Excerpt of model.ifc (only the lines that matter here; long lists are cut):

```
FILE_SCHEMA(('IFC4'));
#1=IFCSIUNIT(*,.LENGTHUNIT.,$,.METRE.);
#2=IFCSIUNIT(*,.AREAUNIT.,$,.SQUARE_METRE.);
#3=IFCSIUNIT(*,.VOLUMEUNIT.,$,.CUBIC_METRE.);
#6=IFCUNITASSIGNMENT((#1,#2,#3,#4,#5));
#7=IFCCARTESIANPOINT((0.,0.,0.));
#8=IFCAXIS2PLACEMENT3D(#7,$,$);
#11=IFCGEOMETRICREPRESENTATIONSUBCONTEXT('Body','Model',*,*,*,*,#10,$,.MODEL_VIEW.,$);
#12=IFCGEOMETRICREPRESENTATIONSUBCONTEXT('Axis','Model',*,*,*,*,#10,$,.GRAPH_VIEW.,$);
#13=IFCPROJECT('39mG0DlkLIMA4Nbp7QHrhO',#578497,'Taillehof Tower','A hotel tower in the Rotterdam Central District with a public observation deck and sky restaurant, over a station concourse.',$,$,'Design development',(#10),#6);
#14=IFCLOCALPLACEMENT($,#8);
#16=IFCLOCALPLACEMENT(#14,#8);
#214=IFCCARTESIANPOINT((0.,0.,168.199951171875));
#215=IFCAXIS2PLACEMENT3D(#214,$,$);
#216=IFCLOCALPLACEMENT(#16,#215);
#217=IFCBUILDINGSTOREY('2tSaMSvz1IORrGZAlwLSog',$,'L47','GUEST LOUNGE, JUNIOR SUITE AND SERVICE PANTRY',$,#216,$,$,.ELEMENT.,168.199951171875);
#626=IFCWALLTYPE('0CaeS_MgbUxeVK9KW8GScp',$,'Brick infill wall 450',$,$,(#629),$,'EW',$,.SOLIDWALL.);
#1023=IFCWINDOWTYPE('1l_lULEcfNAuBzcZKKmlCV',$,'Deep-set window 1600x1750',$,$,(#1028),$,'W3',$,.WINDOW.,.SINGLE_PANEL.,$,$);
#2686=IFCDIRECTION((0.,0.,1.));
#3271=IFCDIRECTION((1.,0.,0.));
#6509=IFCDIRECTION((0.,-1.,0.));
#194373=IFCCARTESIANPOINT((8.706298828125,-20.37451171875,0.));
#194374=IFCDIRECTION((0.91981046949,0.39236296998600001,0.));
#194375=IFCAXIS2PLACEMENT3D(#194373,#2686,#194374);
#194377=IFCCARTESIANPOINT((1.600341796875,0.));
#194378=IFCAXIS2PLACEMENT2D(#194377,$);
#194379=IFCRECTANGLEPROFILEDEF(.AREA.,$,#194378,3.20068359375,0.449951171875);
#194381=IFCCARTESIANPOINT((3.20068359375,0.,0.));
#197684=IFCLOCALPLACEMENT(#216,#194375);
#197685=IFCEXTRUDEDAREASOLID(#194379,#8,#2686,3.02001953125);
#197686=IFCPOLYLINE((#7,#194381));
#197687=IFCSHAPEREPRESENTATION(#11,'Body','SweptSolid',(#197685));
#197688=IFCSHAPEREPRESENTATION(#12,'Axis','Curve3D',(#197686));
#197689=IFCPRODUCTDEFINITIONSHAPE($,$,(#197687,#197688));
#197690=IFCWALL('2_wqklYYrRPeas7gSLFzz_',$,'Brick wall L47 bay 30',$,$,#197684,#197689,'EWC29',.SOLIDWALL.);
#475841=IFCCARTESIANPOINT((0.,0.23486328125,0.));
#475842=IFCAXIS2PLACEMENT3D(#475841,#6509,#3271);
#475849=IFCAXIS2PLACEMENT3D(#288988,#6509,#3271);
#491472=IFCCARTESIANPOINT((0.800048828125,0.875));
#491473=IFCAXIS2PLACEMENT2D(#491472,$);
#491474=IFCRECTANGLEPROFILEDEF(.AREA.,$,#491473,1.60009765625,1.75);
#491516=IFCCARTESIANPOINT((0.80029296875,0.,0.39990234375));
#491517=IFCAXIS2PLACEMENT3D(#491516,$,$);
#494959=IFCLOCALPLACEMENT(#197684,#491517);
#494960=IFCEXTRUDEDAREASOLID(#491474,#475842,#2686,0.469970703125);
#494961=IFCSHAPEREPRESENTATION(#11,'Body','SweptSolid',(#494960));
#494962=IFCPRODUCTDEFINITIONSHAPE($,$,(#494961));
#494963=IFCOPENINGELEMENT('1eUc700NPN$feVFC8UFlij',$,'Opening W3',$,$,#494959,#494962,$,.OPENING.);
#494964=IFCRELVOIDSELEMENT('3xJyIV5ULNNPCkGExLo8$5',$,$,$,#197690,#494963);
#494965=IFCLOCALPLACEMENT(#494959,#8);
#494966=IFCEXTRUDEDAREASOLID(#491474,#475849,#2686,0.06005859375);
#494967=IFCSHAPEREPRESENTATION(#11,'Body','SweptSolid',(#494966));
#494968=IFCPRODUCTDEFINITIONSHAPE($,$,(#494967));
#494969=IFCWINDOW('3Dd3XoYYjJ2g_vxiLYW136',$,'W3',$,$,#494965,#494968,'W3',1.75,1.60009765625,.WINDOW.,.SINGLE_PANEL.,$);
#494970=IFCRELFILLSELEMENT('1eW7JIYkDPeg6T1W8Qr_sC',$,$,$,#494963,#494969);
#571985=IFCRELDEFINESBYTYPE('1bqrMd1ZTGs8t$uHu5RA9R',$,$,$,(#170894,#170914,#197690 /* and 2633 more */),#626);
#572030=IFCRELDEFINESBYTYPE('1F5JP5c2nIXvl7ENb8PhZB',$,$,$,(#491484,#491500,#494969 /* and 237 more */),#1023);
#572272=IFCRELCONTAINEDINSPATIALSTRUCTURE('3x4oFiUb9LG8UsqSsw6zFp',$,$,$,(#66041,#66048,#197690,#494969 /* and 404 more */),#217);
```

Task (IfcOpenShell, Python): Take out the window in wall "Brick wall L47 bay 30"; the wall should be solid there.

```python
import ifcopenshell
import ifcopenshell.api.feature
import ifcopenshell.api.root
import ifcopenshell.geom
import ifcopenshell.util.shape

model = ifcopenshell.open("model.ifc")
settings = ifcopenshell.geom.settings()


def volume(element):
    """Net volume in cubic metres, openings subtracted."""
    shape = ifcopenshell.geom.create_shape(settings, element)
    return ifcopenshell.util.shape.get_volume(shape.geometry)


window = model.by_guid("3Dd3XoYYjJ2g_vxiLYW136")
opening = window.FillsVoids[0].RelatingOpeningElement
wall = opening.VoidsElements[0].RelatingBuildingElement
before = volume(wall)

ifcopenshell.api.root.remove_product(model, product=window)
ifcopenshell.api.feature.remove_feature(model, feature=opening)

after = volume(wall)

print(f"wall volume {before:.3f} -> {after:.3f} m3")

model.write("model-out.ifc")
```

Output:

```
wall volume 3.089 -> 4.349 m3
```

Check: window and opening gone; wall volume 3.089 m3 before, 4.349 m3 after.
